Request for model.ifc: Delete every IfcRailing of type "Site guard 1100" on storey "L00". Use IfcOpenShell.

First a look at what the model holds.

```python
import ifcopenshell
import ifcopenshell.util.element

model = ifcopenshell.open("model.ifc")
print(model.schema)
storey = next(s for s in model.by_type("IfcBuildingStorey") if s.Name == "L00")
railings = [e for e in ifcopenshell.util.element.get_decomposition(storey) if e.is_a("IfcRailing")]
seen = {}
for e in railings:
    element_type = ifcopenshell.util.element.get_type(e)
    name = element_type.Name if element_type not in (None, e) else None
    seen[name] = seen.get(name, 0) + 1
for name, count in sorted(seen.items(), key=str):
    print(count, "x", name)
```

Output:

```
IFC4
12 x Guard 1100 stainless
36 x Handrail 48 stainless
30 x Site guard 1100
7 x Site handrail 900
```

```python
import ifcopenshell
import ifcopenshell.api.root
import ifcopenshell.util.element

model = ifcopenshell.open("model.ifc")

storey = next(s for s in model.by_type("IfcBuildingStorey") if s.Name == "L00")
railings = [e for e in ifcopenshell.util.element.get_decomposition(storey) if e.is_a("IfcRailing")]
targets = [e for e in railings if (t := ifcopenshell.util.element.get_type(e)) not in (None, e) and t.Name == "Site guard 1100"]

for e in targets:
    ifcopenshell.api.root.remove_product(model, product=e)
print(len(targets), "removed")

model.write("model-out.ifc")
```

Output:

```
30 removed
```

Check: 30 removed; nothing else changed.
